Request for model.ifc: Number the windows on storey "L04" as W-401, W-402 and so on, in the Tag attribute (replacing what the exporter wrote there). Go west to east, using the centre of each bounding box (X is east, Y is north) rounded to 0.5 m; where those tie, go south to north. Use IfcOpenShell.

First a look at what the model holds.

```python
import ifcopenshell
import ifcopenshell.util.element
import ifcopenshell.util.placement

model = ifcopenshell.open("model.ifc")
print(model.schema)
storey = next(s for s in model.by_type("IfcBuildingStorey") if s.Name == "L04")
windows = [e for e in ifcopenshell.util.element.get_decomposition(storey) if e.is_a("IfcWindow")]
for e in sorted(windows, key=lambda e: e.id()):
    origin = ifcopenshell.util.placement.get_local_placement(e.ObjectPlacement)[:3, 3]
    print(e.id(), e.Tag, e.Name, origin.round(2) + 0.0, sep=" | ")
```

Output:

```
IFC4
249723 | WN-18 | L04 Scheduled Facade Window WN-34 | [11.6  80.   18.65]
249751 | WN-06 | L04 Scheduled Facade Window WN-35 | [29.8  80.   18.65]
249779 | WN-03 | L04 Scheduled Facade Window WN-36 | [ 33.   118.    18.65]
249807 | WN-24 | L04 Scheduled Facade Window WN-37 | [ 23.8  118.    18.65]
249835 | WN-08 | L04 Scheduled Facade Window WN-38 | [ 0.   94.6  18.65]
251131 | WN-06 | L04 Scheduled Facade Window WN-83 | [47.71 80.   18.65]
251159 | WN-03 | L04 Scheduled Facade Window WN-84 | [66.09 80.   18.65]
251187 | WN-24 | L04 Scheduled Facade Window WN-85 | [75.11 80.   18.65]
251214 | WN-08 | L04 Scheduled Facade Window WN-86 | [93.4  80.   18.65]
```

```python
import ifcopenshell
import ifcopenshell.geom
import ifcopenshell.util.element
import ifcopenshell.util.shape

model = ifcopenshell.open("model.ifc")
settings = ifcopenshell.geom.settings()
settings.set("use-world-coords", True)


def centre(element):
    shape = ifcopenshell.geom.create_shape(settings, element)
    return ifcopenshell.util.shape.get_bbox_centroid(shape.geometry)


storey = next(s for s in model.by_type("IfcBuildingStorey") if s.Name == "L04")
windows = [e for e in ifcopenshell.util.element.get_decomposition(storey) if e.is_a("IfcWindow")]

# Insertion points can sit at a corner or the storey origin, so sort by the geometry (in metres).
centres = {e: centre(e) for e in windows}
windows.sort(key=lambda e: (round(centres[e][0] / 0.5), centres[e][1]))

for i, e in enumerate(windows, start=1):
    number = f"W-4{i:02d}"
    e.Tag = number
    print(e.id(), number)

model.write("model_v2.ifc")
```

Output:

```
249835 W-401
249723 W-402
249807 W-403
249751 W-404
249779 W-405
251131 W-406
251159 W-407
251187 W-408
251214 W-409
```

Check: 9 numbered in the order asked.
